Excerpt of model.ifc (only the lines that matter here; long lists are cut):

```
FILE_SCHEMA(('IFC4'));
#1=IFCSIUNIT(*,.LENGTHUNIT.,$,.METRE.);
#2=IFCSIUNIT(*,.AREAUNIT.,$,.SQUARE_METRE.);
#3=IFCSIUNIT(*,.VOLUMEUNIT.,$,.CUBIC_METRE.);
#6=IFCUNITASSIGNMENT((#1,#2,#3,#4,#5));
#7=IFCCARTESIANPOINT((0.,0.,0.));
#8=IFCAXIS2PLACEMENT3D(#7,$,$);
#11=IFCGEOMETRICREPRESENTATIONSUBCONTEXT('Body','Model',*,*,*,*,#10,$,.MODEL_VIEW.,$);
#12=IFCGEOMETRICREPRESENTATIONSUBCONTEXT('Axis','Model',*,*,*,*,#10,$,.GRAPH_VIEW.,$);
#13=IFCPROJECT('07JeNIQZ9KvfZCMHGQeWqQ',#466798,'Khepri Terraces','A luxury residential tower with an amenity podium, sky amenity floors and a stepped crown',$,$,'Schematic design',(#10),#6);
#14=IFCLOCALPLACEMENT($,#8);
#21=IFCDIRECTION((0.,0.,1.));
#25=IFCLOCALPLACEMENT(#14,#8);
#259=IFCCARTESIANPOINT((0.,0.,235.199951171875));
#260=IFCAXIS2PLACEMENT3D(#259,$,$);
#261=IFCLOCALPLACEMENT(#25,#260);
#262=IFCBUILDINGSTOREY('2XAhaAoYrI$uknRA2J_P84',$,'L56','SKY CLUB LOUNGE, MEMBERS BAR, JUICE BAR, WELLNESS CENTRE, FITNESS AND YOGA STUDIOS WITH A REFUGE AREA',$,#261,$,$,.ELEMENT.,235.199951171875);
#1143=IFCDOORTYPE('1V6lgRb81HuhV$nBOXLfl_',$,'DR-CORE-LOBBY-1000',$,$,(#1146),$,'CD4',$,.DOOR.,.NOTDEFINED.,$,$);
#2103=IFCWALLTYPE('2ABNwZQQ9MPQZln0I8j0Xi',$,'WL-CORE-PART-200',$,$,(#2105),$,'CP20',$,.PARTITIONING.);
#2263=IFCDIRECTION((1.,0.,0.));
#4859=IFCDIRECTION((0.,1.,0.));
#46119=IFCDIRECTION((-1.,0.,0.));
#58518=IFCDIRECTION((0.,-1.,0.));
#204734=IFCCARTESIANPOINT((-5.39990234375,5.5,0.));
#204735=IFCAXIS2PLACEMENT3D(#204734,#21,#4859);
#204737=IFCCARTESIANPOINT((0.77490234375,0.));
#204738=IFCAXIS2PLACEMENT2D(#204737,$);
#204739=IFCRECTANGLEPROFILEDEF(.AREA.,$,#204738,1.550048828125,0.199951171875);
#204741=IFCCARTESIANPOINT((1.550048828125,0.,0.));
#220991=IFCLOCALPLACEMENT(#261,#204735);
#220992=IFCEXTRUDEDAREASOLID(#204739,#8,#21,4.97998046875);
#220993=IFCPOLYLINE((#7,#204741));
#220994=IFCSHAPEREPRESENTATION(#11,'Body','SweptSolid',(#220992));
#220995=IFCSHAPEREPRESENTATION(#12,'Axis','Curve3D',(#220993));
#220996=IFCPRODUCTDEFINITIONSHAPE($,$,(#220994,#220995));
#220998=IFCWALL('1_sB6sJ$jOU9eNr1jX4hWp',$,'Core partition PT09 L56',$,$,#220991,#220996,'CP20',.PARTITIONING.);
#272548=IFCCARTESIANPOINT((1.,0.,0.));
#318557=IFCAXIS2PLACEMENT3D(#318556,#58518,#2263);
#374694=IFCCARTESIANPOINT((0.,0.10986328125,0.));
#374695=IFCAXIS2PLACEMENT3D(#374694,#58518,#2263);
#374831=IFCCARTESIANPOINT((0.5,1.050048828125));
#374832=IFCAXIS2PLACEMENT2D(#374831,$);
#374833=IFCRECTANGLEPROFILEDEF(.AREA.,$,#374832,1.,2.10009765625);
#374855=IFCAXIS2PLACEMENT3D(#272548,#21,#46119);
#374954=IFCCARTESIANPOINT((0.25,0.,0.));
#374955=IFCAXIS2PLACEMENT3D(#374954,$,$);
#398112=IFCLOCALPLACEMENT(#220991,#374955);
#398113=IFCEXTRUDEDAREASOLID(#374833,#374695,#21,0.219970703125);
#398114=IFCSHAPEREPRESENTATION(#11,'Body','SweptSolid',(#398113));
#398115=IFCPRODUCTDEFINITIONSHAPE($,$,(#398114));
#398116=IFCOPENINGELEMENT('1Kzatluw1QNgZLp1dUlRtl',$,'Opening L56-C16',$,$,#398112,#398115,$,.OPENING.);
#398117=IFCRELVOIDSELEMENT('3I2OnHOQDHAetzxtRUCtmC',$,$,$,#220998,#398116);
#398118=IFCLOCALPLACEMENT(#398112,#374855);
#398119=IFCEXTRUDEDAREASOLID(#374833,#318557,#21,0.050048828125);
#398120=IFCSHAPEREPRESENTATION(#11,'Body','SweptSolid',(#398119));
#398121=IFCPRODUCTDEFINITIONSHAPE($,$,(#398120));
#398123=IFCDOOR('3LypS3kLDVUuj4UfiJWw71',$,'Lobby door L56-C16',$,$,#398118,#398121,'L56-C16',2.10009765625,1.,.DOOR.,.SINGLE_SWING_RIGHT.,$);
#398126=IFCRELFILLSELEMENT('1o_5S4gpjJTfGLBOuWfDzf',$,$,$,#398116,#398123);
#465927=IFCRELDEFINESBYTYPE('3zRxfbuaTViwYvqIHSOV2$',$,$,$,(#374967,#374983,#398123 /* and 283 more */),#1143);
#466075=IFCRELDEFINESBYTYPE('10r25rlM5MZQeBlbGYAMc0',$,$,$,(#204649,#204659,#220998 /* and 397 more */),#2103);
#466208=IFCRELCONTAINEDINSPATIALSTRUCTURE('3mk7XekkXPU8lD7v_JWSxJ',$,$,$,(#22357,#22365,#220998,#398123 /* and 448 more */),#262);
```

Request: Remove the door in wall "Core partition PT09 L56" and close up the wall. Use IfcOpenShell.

```python
import ifcopenshell
import ifcopenshell.api.feature
import ifcopenshell.api.root
import ifcopenshell.geom
import ifcopenshell.util.shape

model = ifcopenshell.open("model.ifc")
settings = ifcopenshell.geom.settings()


def volume(element):
    """Net volume in cubic metres, openings subtracted."""
    shape = ifcopenshell.geom.create_shape(settings, element)
    return ifcopenshell.util.shape.get_volume(shape.geometry)


door = model.by_guid("3LypS3kLDVUuj4UfiJWw71")
opening = door.FillsVoids[0].RelatingOpeningElement
wall = opening.VoidsElements[0].RelatingBuildingElement
before = volume(wall)

ifcopenshell.api.root.remove_product(model, product=door)
ifcopenshell.api.feature.remove_feature(model, feature=opening)

after = volume(wall)

print(f"wall volume {before:.3f} -> {after:.3f} m3")

model.write("model_v2.ifc")
```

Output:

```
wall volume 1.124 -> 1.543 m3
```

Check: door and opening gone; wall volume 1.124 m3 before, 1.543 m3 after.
